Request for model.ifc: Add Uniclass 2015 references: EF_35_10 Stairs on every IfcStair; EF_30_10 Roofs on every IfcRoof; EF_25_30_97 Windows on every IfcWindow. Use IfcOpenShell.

First a look at what the model holds.

```python
import ifcopenshell

model = ifcopenshell.open("model.ifc")
print(model.schema)
print("classifications:", [c.Name for c in model.by_type("IfcClassification")])
for ifc_class in ("IfcDoor", "IfcRoof", "IfcStair", "IfcWall", "IfcWindow"):
    print(ifc_class, len(model.by_type(ifc_class)))
```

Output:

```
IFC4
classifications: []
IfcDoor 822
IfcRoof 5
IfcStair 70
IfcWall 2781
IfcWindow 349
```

```python
import ifcopenshell
import ifcopenshell.api.classification

model = ifcopenshell.open("model.ifc")

system = ifcopenshell.api.classification.add_classification(model, classification="Uniclass 2015")

codes = {
    "IfcStair": ("EF_35_10", "Stairs"),
    "IfcRoof": ("EF_30_10", "Roofs"),
    "IfcWindow": ("EF_25_30_97", "Windows"),
}
for ifc_class, (code, name) in codes.items():
    products = model.by_type(ifc_class)
    ifcopenshell.api.classification.add_reference(
        model, products=products, classification=system, identification=code, name=name
    )
    print(code, len(products))

model.write("model_updated.ifc")
```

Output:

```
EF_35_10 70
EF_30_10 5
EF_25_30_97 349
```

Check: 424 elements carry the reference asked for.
